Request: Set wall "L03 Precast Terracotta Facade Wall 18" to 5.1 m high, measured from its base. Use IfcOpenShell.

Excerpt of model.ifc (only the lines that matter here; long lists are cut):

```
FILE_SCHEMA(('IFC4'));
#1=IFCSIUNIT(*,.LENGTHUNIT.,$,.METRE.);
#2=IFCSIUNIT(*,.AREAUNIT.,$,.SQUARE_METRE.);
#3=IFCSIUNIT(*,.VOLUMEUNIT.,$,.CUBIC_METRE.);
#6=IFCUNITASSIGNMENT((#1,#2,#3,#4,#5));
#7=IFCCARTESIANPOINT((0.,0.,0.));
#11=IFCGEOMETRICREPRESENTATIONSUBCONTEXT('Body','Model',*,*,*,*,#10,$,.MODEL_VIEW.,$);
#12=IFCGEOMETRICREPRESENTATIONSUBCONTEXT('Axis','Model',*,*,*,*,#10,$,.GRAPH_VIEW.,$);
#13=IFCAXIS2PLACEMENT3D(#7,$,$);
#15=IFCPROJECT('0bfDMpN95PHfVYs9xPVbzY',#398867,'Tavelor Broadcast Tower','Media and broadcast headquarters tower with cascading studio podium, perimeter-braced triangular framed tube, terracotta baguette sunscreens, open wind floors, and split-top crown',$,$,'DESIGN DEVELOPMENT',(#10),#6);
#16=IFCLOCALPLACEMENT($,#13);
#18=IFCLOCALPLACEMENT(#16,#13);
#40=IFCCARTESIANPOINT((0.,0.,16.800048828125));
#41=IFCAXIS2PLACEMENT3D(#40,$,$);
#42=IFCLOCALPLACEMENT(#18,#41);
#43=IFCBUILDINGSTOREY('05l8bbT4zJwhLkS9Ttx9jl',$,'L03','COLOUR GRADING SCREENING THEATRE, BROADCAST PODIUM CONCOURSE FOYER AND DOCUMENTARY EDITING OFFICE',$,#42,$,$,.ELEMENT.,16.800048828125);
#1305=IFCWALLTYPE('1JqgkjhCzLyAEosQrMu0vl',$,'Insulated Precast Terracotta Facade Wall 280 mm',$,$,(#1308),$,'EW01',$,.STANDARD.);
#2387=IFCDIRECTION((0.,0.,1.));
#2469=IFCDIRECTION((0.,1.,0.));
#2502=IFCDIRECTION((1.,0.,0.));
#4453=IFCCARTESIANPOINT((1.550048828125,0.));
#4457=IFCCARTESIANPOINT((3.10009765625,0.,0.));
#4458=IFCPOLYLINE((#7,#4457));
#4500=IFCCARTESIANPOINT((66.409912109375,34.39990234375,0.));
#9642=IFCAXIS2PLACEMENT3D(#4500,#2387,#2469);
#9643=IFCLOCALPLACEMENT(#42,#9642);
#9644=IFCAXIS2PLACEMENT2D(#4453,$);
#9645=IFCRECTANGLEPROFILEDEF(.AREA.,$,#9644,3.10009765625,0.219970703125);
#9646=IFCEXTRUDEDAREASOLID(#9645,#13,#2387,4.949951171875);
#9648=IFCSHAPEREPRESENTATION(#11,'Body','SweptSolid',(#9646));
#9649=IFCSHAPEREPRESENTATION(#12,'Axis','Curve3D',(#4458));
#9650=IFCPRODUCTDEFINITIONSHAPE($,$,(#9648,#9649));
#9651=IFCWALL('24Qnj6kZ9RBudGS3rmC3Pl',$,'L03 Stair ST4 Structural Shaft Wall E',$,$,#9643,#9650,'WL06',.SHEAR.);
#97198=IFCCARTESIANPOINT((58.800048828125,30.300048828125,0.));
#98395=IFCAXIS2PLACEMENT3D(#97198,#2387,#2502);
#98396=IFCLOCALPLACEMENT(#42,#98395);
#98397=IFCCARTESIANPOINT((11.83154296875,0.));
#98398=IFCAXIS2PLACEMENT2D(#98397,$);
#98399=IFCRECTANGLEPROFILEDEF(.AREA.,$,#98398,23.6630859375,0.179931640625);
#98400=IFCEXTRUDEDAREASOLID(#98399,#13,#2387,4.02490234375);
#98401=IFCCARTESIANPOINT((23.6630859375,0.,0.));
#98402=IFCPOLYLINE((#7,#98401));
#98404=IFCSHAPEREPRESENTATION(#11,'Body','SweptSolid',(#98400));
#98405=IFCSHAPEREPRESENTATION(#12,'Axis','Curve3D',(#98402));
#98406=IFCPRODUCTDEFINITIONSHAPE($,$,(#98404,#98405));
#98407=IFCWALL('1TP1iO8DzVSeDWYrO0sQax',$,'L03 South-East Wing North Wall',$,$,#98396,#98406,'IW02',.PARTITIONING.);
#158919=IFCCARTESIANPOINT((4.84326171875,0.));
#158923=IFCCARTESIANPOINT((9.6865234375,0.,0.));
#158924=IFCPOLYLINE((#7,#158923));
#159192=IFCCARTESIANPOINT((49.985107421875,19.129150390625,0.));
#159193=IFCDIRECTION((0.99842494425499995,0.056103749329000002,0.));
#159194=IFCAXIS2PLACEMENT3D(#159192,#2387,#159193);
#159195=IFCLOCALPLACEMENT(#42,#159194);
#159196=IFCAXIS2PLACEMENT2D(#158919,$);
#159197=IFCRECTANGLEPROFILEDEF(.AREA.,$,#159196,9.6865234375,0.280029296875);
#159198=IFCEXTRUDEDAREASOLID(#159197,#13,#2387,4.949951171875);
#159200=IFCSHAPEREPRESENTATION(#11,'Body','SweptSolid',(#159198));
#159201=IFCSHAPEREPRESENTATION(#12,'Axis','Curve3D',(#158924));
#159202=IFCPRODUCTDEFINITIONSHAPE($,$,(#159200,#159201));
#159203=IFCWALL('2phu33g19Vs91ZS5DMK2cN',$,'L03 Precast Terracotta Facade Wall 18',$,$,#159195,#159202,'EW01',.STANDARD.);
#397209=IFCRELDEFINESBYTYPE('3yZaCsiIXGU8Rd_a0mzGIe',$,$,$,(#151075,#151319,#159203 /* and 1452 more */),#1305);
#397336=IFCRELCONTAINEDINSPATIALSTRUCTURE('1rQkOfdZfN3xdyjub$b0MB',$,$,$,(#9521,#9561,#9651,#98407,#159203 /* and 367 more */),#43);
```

```python
import ifcopenshell
import ifcopenshell.geom
import ifcopenshell.util.representation
import ifcopenshell.util.shape
import ifcopenshell.util.unit

model = ifcopenshell.open("model.ifc")
unit_scale = ifcopenshell.util.unit.calculate_unit_scale(model)
settings = ifcopenshell.geom.settings()


def volume(element):
    """Net volume in cubic metres, openings subtracted."""
    shape = ifcopenshell.geom.create_shape(settings, element)
    return ifcopenshell.util.shape.get_volume(shape.geometry)


wall = model.by_guid("2phu33g19Vs91ZS5DMK2cN")
before = volume(wall)

body = ifcopenshell.util.representation.get_representation(wall, "Model", "Body")
solid = body.Items[0]
old_height = solid.Depth
solid.Depth = 5.1 / unit_scale
after = volume(wall)

print(f"height {old_height:g} -> {solid.Depth:g}, volume {before:.3f} -> {after:.3f} m3")

model.write("model_edited.ifc")
```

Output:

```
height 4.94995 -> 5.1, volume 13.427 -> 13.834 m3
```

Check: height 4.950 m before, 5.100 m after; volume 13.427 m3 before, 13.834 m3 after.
